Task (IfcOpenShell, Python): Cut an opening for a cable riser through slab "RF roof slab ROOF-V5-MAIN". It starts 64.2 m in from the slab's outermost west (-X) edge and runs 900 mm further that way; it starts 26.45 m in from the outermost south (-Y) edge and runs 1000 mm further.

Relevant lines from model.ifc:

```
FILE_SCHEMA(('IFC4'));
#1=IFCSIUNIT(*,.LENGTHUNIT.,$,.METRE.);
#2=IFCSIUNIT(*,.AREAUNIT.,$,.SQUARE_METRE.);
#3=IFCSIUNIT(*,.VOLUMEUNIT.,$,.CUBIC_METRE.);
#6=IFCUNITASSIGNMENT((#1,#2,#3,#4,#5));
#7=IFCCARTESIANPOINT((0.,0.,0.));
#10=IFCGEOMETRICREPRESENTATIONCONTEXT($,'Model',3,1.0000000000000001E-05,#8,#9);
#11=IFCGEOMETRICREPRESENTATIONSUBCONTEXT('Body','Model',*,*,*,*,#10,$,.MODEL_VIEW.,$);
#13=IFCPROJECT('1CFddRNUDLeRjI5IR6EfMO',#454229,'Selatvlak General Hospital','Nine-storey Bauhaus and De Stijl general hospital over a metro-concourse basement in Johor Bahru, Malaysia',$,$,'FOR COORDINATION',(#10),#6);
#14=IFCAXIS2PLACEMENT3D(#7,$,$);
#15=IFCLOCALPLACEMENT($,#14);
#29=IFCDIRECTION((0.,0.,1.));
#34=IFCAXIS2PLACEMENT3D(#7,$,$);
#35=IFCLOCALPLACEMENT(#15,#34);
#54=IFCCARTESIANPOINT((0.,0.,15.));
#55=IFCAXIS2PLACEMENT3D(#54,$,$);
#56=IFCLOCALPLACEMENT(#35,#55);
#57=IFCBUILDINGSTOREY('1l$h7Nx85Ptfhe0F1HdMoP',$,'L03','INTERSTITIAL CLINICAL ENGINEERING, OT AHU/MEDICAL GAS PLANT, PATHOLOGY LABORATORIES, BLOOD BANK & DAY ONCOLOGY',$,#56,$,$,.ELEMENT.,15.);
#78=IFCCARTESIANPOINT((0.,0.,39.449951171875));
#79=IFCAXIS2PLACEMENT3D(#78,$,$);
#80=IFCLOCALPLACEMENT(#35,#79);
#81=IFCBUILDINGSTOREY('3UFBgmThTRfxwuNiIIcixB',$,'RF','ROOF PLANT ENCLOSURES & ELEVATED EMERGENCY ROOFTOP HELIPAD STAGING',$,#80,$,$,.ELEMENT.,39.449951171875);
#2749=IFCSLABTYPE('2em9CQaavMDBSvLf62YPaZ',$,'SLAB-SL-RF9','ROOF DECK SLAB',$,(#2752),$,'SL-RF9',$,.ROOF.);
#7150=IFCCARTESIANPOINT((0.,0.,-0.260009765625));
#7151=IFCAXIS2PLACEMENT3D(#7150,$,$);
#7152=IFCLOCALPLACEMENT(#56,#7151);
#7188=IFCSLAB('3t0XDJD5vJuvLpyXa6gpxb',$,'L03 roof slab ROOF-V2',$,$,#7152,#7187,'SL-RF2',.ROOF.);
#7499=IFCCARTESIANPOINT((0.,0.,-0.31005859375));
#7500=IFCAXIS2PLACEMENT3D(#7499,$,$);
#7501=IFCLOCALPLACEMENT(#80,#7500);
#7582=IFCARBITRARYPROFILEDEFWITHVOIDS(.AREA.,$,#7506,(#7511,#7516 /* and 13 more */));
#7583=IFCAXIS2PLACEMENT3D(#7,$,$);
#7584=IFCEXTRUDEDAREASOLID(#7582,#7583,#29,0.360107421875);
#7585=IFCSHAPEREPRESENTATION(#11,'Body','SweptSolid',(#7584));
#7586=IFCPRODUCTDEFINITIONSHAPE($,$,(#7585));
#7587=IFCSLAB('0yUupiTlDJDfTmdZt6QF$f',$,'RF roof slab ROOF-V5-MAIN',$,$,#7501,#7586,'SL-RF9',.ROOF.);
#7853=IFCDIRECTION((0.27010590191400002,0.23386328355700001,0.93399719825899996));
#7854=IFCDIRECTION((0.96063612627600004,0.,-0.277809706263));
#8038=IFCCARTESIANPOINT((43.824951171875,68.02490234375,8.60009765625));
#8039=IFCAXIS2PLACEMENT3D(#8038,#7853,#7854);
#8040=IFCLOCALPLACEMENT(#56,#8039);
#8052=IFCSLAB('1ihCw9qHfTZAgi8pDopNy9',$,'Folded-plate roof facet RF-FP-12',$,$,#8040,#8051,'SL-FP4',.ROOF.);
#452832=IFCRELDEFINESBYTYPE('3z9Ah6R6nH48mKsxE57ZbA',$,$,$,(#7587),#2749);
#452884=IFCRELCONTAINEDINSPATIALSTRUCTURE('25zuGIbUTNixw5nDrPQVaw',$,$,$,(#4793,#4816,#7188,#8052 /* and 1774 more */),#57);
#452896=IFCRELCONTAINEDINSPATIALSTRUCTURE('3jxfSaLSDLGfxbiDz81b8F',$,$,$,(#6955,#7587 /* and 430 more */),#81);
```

```python
import numpy as np
import ifcopenshell
import ifcopenshell.api.feature
import ifcopenshell.api.geometry
import ifcopenshell.api.root
import ifcopenshell.geom
import ifcopenshell.util.placement
import ifcopenshell.util.representation
import ifcopenshell.util.shape
import ifcopenshell.util.unit

model = ifcopenshell.open("model.ifc")
unit_scale = ifcopenshell.util.unit.calculate_unit_scale(model)
settings = ifcopenshell.geom.settings()


def volume(element):
    """Net volume in cubic metres, openings subtracted."""
    shape = ifcopenshell.geom.create_shape(settings, element)
    return ifcopenshell.util.shape.get_volume(shape.geometry)


slab = model.by_id(7587)
before = volume(slab)

# Extent in the slab's own axes, in metres. The edges named are its -X and -Y sides.
slab_shape = ifcopenshell.geom.create_shape(settings, slab)
vertices = ifcopenshell.util.shape.get_vertices(slab_shape.geometry)
x_min, y_min, bottom = vertices.min(axis=0)
top = vertices[:, 2].max()

opening = ifcopenshell.api.root.create_entity(model, ifc_class="IfcOpeningElement", name="Cable riser opening", predefined_type="OPENING")
context = ifcopenshell.util.representation.get_context(model, "Model", "Body", "MODEL_VIEW")
width, depth = 0.9, 1
outline = [(0.0, 0.0), (width, 0.0), (width, depth), (0.0, depth), (0.0, 0.0)]
# Overshoot both faces by 50 mm so the cut is clean.
shape = ifcopenshell.api.geometry.add_slab_representation(
    model, context=context, depth=top - bottom + 0.1, polyline=outline
)
ifcopenshell.api.geometry.assign_representation(model, product=opening, representation=shape)

matrix = ifcopenshell.util.placement.get_local_placement(slab.ObjectPlacement)
matrix[:, 3] = matrix @ np.append(np.array([x_min + 64.2, y_min + 26.45, bottom - 0.05]) / unit_scale, 1.0)
ifcopenshell.api.geometry.edit_object_placement(model, product=opening, matrix=matrix, is_si=False)
ifcopenshell.api.feature.add_feature(model, feature=opening, element=slab)

after = volume(slab)

print(f"slab volume {before:.3f} -> {after:.3f} m3")

model.write("model-out.ifc")
```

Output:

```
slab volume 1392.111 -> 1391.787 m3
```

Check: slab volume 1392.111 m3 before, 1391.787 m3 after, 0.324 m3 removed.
